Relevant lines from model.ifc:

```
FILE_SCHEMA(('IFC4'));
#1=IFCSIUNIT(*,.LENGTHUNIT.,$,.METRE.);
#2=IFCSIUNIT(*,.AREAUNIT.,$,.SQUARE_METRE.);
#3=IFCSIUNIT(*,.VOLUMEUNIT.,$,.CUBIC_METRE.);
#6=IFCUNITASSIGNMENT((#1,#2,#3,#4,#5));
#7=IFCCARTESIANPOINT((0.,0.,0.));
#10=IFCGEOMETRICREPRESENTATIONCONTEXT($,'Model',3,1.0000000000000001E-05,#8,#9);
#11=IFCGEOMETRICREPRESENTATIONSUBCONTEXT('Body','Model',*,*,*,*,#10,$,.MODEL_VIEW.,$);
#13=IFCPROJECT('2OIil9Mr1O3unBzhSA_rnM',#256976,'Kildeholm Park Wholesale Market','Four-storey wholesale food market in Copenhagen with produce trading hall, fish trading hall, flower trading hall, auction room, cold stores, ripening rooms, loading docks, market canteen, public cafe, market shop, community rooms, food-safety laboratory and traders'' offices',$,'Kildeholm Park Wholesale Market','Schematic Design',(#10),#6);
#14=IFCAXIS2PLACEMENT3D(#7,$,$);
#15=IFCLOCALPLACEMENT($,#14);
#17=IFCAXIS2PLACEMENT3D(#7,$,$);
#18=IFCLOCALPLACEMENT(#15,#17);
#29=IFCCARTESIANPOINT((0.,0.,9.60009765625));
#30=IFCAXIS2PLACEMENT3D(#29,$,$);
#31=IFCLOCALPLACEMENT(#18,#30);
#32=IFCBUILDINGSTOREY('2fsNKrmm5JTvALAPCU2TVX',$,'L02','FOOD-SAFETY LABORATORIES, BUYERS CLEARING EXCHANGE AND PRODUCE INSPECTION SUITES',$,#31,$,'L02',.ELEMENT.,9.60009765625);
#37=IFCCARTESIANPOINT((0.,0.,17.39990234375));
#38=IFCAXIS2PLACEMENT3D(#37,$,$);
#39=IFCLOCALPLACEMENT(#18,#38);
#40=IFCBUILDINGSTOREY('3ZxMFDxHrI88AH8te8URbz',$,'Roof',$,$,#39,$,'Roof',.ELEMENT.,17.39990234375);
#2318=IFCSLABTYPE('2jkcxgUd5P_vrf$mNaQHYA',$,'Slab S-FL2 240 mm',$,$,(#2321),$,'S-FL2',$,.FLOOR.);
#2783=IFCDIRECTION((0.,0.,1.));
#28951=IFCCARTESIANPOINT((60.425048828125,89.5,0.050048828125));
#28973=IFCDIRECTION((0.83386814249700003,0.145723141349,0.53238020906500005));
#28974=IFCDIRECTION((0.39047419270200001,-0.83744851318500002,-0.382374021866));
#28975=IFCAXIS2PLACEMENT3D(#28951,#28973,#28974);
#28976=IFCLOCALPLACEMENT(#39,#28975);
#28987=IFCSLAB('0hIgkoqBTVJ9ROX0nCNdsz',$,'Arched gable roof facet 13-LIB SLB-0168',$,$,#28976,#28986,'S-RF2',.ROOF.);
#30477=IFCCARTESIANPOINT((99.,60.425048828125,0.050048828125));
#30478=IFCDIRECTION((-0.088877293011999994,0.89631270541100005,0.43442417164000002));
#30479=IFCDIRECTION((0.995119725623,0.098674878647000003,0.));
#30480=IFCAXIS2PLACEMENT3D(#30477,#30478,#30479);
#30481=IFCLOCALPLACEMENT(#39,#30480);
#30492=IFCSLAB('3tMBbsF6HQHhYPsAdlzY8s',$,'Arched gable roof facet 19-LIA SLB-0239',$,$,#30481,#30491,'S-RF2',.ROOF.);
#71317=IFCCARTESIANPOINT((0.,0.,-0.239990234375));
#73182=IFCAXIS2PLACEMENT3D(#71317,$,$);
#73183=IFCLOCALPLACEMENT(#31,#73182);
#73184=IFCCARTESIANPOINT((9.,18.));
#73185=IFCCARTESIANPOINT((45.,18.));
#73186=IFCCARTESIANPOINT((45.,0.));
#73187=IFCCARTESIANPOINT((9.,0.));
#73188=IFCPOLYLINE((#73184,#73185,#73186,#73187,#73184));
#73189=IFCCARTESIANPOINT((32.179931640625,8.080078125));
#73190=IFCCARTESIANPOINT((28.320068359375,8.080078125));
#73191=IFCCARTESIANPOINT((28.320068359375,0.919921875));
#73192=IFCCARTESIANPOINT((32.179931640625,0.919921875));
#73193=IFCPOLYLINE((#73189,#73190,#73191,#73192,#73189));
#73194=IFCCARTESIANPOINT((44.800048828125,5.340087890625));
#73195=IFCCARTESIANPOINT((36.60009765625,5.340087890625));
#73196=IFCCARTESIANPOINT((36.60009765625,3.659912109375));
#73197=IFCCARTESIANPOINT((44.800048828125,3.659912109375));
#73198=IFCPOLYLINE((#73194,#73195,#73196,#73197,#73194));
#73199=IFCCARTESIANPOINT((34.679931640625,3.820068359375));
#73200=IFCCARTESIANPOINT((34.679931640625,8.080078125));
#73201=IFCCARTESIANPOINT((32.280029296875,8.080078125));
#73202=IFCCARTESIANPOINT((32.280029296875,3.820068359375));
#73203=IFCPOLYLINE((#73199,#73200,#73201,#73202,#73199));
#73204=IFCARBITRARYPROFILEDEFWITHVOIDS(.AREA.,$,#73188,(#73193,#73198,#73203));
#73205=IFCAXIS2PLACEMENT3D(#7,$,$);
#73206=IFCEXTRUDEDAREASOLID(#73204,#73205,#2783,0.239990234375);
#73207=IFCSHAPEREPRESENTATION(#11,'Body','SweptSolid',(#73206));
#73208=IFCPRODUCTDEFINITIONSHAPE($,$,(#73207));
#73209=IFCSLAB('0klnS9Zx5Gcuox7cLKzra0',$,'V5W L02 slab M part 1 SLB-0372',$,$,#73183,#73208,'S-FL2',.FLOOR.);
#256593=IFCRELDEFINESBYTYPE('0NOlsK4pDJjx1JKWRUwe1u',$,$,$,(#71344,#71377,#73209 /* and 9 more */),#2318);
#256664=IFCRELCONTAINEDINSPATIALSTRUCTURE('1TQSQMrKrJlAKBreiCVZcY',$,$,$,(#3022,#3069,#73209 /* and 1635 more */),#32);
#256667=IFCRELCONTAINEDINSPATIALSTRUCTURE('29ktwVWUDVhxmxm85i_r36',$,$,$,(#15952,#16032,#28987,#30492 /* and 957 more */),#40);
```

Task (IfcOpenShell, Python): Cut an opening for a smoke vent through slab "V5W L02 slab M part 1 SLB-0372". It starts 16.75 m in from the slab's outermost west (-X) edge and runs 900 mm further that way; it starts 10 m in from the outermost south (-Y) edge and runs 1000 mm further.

```python
import numpy as np
import ifcopenshell
import ifcopenshell.api.feature
import ifcopenshell.api.geometry
import ifcopenshell.api.root
import ifcopenshell.geom
import ifcopenshell.util.placement
import ifcopenshell.util.representation
import ifcopenshell.util.shape
import ifcopenshell.util.unit

model = ifcopenshell.open("model.ifc")
unit_scale = ifcopenshell.util.unit.calculate_unit_scale(model)
settings = ifcopenshell.geom.settings()


def volume(element):
    """Net volume in cubic metres, openings subtracted."""
    shape = ifcopenshell.geom.create_shape(settings, element)
    return ifcopenshell.util.shape.get_volume(shape.geometry)


slab = model.by_guid("0klnS9Zx5Gcuox7cLKzra0")
before = volume(slab)

# Extent in the slab's own axes, in metres. The edges named are its -X and -Y sides.
slab_shape = ifcopenshell.geom.create_shape(settings, slab)
vertices = ifcopenshell.util.shape.get_vertices(slab_shape.geometry)
x_min, y_min, bottom = vertices.min(axis=0)
top = vertices[:, 2].max()

opening = ifcopenshell.api.root.create_entity(model, ifc_class="IfcOpeningElement", name="Smoke vent opening", predefined_type="OPENING")
context = ifcopenshell.util.representation.get_context(model, "Model", "Body", "MODEL_VIEW")
width, depth = 0.9, 1
outline = [(0.0, 0.0), (width, 0.0), (width, depth), (0.0, depth), (0.0, 0.0)]
# Overshoot both faces by 50 mm so the cut is clean.
shape = ifcopenshell.api.geometry.add_slab_representation(
    model, context=context, depth=top - bottom + 0.1, polyline=outline
)
ifcopenshell.api.geometry.assign_representation(model, product=opening, representation=shape)

matrix = ifcopenshell.util.placement.get_local_placement(slab.ObjectPlacement)
matrix[:, 3] = matrix @ np.append(np.array([x_min + 16.75, y_min + 10, bottom - 0.05]) / unit_scale, 1.0)
ifcopenshell.api.geometry.edit_object_placement(model, product=opening, matrix=matrix, is_si=False)
ifcopenshell.api.feature.add_feature(model, feature=opening, element=slab)

after = volume(slab)

print(f"slab volume {before:.3f} -> {after:.3f} m3")

model.write("model_updated.ifc")
```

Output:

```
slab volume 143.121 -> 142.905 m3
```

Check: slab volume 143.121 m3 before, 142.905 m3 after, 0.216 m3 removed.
